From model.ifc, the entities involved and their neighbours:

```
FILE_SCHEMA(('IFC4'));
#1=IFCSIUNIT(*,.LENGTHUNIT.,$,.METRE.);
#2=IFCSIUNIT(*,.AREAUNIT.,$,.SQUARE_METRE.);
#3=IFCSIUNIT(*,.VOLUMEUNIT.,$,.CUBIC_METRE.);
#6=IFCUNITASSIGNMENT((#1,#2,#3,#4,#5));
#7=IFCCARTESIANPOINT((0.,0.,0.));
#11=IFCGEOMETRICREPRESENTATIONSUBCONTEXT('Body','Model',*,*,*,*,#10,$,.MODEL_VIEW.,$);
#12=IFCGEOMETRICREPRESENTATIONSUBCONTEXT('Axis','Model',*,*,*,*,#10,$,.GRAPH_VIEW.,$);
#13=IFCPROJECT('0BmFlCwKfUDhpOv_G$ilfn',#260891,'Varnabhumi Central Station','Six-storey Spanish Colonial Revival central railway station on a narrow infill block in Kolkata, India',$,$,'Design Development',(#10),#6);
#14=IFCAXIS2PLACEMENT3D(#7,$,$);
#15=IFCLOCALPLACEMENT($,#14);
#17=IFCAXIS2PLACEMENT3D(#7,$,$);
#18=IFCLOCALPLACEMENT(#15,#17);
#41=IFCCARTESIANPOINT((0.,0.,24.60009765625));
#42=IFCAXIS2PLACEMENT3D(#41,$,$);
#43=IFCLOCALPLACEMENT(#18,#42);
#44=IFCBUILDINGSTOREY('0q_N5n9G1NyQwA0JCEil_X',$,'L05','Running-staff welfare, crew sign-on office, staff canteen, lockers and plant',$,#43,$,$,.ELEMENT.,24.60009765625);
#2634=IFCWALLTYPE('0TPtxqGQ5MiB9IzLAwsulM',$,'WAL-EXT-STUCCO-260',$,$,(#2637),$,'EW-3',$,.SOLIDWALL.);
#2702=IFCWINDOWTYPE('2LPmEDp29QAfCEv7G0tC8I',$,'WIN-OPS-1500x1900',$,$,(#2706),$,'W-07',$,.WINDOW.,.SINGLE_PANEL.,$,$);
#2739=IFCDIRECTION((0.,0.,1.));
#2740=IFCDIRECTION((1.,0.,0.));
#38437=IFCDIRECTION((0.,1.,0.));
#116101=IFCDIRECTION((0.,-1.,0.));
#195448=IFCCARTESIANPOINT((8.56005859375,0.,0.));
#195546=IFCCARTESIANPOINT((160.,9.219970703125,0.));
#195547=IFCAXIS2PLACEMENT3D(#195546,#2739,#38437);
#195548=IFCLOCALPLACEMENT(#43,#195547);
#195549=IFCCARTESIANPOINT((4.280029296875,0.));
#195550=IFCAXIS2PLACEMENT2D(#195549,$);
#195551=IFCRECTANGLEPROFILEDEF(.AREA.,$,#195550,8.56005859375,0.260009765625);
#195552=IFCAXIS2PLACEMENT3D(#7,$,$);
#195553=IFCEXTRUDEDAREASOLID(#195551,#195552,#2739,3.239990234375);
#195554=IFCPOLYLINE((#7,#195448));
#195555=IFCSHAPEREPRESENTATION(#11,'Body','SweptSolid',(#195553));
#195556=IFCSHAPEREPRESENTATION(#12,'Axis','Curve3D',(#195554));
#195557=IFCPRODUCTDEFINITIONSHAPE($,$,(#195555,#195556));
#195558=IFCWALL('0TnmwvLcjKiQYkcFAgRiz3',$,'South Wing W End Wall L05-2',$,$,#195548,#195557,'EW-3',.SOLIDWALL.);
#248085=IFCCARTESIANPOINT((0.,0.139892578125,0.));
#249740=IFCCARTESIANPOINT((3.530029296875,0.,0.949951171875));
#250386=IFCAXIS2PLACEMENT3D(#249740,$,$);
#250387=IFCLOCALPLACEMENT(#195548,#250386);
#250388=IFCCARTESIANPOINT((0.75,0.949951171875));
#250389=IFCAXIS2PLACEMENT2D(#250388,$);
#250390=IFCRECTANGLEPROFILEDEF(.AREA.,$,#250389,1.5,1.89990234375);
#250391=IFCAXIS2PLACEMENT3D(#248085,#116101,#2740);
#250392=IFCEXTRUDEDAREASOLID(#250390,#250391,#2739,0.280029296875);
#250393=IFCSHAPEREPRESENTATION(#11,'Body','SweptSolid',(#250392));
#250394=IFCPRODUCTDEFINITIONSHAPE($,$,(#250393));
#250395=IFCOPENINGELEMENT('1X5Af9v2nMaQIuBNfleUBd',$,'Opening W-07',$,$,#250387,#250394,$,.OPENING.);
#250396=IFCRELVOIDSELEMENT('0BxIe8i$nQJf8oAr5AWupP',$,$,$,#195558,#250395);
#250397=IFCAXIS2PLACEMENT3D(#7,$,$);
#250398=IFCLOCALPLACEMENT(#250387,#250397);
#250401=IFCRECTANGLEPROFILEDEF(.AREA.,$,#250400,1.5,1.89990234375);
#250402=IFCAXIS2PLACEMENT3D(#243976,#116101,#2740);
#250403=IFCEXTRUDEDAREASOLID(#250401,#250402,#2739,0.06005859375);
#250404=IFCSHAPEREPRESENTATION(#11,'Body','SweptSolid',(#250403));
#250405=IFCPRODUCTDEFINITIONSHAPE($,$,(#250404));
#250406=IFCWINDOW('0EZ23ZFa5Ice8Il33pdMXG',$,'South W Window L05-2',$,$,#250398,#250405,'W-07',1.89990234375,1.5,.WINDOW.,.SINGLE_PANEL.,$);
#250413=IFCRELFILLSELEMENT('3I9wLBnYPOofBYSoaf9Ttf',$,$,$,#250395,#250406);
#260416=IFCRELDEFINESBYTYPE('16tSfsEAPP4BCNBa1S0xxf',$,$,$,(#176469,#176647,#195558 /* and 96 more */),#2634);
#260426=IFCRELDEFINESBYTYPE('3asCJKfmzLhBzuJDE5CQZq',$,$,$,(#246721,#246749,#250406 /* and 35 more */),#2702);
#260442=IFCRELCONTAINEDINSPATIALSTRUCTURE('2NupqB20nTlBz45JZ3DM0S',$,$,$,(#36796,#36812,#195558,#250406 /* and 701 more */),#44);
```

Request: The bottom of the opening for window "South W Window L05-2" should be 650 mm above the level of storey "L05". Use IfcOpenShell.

```python
import numpy as np
import ifcopenshell
import ifcopenshell.api.geometry
import ifcopenshell.geom
import ifcopenshell.util.element
import ifcopenshell.util.placement
import ifcopenshell.util.shape
import ifcopenshell.util.unit

model = ifcopenshell.open("model.ifc")
unit_scale = ifcopenshell.util.unit.calculate_unit_scale(model)

window = model.by_id(250406)
opening = window.FillsVoids[0].RelatingOpeningElement
storey = ifcopenshell.util.element.get_container(window, ifc_class="IfcBuildingStorey")
level = ifcopenshell.util.placement.get_local_placement(storey.ObjectPlacement)[2, 3]

# The opening's origin need not be at the sill, so measure its lowest point.
shape = ifcopenshell.geom.create_shape(ifcopenshell.geom.settings(), opening)
bottom = ifcopenshell.util.shape.get_shape_bottom_elevation(shape, shape.geometry) / unit_scale
dz = level + 0.65 / unit_scale - bottom

shift = np.array([0.0, 0.0, dz])
# The window is placed relative to its opening, so it follows when the opening moves.
matrix = ifcopenshell.util.placement.get_local_placement(opening.ObjectPlacement)
matrix[:3, 3] += shift
ifcopenshell.api.geometry.edit_object_placement(
    model, product=opening, matrix=matrix, is_si=False, should_transform_children=True
)

print(f"moved by {dz * unit_scale:+.3f} m")

model.write("model_updated.ifc")
```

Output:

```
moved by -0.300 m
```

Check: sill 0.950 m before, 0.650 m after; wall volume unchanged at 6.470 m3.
